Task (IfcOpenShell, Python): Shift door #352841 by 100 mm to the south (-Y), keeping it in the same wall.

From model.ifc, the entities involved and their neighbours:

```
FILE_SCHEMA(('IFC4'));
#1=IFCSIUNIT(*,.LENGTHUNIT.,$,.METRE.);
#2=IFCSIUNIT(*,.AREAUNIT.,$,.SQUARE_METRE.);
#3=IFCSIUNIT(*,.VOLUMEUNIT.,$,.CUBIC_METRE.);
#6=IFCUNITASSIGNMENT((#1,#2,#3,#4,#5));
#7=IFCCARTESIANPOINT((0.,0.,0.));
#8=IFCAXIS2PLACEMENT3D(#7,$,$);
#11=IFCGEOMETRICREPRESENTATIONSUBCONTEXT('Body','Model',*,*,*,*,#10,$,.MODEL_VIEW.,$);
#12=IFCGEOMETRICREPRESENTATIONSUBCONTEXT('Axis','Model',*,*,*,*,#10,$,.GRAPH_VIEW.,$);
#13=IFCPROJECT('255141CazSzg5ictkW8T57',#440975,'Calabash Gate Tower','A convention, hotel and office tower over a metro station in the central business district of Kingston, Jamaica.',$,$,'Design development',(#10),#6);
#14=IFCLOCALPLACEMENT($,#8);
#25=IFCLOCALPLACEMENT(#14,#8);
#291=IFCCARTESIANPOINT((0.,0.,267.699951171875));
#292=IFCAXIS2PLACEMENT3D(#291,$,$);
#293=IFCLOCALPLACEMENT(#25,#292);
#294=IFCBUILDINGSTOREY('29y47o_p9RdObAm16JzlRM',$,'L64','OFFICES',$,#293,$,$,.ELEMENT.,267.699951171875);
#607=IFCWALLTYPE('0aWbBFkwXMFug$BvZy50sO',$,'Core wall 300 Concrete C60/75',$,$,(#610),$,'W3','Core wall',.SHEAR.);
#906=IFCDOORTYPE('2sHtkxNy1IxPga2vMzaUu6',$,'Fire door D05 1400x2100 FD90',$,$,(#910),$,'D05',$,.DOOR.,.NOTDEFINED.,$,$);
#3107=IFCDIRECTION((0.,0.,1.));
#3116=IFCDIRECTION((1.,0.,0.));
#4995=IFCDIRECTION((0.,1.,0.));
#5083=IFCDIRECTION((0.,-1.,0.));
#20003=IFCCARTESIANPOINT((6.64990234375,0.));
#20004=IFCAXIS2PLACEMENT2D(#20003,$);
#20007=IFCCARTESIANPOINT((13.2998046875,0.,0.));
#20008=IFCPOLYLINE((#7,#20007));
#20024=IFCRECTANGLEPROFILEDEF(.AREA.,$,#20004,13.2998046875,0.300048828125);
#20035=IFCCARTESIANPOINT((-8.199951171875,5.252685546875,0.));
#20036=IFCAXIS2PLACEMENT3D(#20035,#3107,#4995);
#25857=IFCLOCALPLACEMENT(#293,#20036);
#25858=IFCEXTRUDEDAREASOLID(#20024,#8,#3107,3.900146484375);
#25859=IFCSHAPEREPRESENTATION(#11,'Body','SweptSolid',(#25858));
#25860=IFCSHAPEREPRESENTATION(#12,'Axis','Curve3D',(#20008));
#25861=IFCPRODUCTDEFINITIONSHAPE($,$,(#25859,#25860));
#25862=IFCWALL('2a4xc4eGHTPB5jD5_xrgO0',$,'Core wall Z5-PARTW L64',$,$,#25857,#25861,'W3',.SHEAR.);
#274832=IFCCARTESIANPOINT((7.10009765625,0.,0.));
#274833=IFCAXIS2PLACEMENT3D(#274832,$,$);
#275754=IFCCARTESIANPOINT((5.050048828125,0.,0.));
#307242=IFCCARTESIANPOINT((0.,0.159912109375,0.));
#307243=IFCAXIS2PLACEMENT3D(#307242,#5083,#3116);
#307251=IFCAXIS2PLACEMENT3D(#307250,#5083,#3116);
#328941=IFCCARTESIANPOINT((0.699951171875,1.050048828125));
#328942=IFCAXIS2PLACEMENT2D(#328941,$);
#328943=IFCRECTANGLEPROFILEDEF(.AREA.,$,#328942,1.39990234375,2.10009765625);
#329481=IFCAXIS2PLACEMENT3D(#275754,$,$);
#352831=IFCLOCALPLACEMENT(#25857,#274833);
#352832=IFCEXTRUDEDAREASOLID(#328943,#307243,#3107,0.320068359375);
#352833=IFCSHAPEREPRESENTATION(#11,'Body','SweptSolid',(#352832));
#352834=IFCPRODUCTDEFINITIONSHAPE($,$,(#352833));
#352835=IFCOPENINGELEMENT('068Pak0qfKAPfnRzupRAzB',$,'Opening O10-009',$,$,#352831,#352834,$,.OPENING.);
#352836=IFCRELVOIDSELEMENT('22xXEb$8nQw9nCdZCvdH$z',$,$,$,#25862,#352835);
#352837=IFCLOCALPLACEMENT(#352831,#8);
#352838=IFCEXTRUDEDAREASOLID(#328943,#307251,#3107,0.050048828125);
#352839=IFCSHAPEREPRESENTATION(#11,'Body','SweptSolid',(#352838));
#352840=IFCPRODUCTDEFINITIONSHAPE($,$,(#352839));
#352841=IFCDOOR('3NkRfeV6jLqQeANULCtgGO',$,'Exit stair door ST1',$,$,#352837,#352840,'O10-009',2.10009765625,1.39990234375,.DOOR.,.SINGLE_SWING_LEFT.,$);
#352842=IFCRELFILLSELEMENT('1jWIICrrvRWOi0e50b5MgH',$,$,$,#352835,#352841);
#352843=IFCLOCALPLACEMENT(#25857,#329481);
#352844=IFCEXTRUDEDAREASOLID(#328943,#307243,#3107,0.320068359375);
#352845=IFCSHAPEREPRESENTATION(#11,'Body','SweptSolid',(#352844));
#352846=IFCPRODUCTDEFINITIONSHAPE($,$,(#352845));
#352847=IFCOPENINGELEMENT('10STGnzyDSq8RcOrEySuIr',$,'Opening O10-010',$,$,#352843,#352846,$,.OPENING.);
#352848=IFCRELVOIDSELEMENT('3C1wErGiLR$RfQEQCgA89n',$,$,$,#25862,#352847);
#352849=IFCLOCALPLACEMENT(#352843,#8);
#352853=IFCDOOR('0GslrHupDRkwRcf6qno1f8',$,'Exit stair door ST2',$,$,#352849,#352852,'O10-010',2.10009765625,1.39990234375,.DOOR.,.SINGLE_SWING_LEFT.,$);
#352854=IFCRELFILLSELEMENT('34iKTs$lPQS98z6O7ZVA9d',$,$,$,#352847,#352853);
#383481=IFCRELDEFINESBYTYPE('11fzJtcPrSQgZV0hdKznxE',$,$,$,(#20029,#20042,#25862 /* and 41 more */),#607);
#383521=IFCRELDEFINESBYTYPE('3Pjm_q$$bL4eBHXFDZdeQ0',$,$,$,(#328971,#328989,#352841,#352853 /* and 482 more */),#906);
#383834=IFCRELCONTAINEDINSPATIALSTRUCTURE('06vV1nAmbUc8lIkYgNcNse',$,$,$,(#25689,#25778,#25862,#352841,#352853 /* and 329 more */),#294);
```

```python
import ifcopenshell
import ifcopenshell.api.geometry
import ifcopenshell.util.placement
import ifcopenshell.util.unit

model = ifcopenshell.open("model.ifc")
unit_scale = ifcopenshell.util.unit.calculate_unit_scale(model)

door = model.by_id(352841)
opening = door.FillsVoids[0].RelatingOpeningElement
wall = opening.VoidsElements[0].RelatingBuildingElement

wall_matrix = ifcopenshell.util.placement.get_local_placement(wall.ObjectPlacement)
shift = wall_matrix[:3, 0] * -0.1 / unit_scale
before = ifcopenshell.util.placement.get_local_placement(door.ObjectPlacement)[:3, 3].copy()

# The door is placed relative to its opening, so it follows when the opening moves.
matrix = ifcopenshell.util.placement.get_local_placement(opening.ObjectPlacement)
matrix[:3, 3] += shift
ifcopenshell.api.geometry.edit_object_placement(
    model, product=opening, matrix=matrix, is_si=False, should_transform_children=True
)

after = ifcopenshell.util.placement.get_local_placement(door.ObjectPlacement)[:3, 3]
print("door moved by", (after - before).round(3) + 0.0)

model.write("model-out.ifc")
```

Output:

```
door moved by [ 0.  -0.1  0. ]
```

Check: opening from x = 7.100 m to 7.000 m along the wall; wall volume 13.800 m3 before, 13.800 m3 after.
